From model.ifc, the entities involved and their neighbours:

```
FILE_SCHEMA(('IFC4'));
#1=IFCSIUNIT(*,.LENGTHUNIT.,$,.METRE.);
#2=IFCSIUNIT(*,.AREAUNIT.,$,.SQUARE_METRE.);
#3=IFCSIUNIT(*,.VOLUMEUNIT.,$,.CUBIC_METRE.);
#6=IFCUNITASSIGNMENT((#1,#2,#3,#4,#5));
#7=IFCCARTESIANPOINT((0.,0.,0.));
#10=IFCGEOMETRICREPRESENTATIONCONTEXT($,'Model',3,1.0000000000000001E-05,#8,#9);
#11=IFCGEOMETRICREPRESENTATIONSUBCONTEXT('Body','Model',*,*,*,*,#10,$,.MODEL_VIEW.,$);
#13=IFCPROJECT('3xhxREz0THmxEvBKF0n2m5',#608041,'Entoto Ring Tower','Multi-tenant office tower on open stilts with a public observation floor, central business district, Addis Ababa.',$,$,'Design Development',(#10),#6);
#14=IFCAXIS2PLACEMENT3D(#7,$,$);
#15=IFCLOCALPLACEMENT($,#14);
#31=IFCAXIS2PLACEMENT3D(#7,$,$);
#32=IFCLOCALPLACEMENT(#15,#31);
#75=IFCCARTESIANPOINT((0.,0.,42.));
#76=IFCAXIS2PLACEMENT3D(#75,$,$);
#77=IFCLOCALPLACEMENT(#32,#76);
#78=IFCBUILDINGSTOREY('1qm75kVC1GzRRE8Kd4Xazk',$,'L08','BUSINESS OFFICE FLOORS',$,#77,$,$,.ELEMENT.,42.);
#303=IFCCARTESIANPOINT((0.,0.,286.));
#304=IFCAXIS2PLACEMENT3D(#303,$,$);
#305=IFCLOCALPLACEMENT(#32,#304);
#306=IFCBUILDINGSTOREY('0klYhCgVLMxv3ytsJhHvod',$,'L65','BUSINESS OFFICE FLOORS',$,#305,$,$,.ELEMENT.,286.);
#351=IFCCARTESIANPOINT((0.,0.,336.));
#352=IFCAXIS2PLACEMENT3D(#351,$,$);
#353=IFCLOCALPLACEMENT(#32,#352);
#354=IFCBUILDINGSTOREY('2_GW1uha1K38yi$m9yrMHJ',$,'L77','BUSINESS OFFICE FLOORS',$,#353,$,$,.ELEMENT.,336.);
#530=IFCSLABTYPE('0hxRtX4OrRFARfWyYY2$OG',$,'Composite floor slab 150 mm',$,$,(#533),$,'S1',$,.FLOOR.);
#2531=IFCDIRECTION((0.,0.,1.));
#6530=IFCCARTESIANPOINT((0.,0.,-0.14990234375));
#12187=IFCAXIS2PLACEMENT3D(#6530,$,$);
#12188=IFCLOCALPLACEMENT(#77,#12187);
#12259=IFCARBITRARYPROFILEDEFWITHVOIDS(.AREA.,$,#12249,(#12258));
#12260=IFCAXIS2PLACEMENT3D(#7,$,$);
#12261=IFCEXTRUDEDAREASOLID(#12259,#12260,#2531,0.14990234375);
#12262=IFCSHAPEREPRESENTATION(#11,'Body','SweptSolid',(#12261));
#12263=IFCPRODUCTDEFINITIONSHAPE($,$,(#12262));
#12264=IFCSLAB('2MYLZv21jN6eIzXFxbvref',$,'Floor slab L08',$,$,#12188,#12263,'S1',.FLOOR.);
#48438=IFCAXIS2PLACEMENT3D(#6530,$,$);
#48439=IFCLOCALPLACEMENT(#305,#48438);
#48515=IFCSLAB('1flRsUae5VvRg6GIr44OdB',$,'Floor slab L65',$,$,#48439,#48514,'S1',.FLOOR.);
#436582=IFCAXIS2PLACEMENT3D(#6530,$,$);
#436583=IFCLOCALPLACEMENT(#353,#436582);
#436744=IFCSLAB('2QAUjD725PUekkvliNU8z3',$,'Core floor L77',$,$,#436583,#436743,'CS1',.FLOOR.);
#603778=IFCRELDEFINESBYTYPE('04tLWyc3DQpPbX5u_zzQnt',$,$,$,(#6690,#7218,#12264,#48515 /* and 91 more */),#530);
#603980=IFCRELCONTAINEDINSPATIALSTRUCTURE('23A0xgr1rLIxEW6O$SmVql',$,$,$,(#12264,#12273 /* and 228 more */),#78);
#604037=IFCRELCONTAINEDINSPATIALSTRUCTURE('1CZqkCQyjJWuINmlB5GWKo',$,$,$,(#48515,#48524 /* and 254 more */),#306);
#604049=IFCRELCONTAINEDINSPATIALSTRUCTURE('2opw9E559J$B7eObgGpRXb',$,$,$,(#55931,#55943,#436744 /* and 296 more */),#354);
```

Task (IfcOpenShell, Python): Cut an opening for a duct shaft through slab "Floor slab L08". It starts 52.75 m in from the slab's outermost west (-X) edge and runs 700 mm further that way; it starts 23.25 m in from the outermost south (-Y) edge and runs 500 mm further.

```python
import numpy as np
import ifcopenshell
import ifcopenshell.api.feature
import ifcopenshell.api.geometry
import ifcopenshell.api.root
import ifcopenshell.geom
import ifcopenshell.util.placement
import ifcopenshell.util.representation
import ifcopenshell.util.shape
import ifcopenshell.util.unit

model = ifcopenshell.open("model.ifc")
unit_scale = ifcopenshell.util.unit.calculate_unit_scale(model)
settings = ifcopenshell.geom.settings()


def volume(element):
    """Net volume in cubic metres, openings subtracted."""
    shape = ifcopenshell.geom.create_shape(settings, element)
    return ifcopenshell.util.shape.get_volume(shape.geometry)


slab = model.by_guid("2MYLZv21jN6eIzXFxbvref")
before = volume(slab)

# Extent in the slab's own axes, in metres. The edges named are its -X and -Y sides.
slab_shape = ifcopenshell.geom.create_shape(settings, slab)
vertices = ifcopenshell.util.shape.get_vertices(slab_shape.geometry)
x_min, y_min, bottom = vertices.min(axis=0)
top = vertices[:, 2].max()

opening = ifcopenshell.api.root.create_entity(model, ifc_class="IfcOpeningElement", name="Duct shaft opening", predefined_type="OPENING")
context = ifcopenshell.util.representation.get_context(model, "Model", "Body", "MODEL_VIEW")
width, depth = 0.7, 0.5
outline = [(0.0, 0.0), (width, 0.0), (width, depth), (0.0, depth), (0.0, 0.0)]
# Overshoot both faces by 50 mm so the cut is clean.
shape = ifcopenshell.api.geometry.add_slab_representation(
    model, context=context, depth=top - bottom + 0.1, polyline=outline
)
ifcopenshell.api.geometry.assign_representation(model, product=opening, representation=shape)

matrix = ifcopenshell.util.placement.get_local_placement(slab.ObjectPlacement)
matrix[:, 3] = matrix @ np.append(np.array([x_min + 52.75, y_min + 23.25, bottom - 0.05]) / unit_scale, 1.0)
ifcopenshell.api.geometry.edit_object_placement(model, product=opening, matrix=matrix, is_si=False)
ifcopenshell.api.feature.add_feature(model, feature=opening, element=slab)

after = volume(slab)

print(f"slab volume {before:.3f} -> {after:.3f} m3")

model.write("model_rev.ifc")
```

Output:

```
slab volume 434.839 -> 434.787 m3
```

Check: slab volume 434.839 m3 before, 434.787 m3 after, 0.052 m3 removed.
